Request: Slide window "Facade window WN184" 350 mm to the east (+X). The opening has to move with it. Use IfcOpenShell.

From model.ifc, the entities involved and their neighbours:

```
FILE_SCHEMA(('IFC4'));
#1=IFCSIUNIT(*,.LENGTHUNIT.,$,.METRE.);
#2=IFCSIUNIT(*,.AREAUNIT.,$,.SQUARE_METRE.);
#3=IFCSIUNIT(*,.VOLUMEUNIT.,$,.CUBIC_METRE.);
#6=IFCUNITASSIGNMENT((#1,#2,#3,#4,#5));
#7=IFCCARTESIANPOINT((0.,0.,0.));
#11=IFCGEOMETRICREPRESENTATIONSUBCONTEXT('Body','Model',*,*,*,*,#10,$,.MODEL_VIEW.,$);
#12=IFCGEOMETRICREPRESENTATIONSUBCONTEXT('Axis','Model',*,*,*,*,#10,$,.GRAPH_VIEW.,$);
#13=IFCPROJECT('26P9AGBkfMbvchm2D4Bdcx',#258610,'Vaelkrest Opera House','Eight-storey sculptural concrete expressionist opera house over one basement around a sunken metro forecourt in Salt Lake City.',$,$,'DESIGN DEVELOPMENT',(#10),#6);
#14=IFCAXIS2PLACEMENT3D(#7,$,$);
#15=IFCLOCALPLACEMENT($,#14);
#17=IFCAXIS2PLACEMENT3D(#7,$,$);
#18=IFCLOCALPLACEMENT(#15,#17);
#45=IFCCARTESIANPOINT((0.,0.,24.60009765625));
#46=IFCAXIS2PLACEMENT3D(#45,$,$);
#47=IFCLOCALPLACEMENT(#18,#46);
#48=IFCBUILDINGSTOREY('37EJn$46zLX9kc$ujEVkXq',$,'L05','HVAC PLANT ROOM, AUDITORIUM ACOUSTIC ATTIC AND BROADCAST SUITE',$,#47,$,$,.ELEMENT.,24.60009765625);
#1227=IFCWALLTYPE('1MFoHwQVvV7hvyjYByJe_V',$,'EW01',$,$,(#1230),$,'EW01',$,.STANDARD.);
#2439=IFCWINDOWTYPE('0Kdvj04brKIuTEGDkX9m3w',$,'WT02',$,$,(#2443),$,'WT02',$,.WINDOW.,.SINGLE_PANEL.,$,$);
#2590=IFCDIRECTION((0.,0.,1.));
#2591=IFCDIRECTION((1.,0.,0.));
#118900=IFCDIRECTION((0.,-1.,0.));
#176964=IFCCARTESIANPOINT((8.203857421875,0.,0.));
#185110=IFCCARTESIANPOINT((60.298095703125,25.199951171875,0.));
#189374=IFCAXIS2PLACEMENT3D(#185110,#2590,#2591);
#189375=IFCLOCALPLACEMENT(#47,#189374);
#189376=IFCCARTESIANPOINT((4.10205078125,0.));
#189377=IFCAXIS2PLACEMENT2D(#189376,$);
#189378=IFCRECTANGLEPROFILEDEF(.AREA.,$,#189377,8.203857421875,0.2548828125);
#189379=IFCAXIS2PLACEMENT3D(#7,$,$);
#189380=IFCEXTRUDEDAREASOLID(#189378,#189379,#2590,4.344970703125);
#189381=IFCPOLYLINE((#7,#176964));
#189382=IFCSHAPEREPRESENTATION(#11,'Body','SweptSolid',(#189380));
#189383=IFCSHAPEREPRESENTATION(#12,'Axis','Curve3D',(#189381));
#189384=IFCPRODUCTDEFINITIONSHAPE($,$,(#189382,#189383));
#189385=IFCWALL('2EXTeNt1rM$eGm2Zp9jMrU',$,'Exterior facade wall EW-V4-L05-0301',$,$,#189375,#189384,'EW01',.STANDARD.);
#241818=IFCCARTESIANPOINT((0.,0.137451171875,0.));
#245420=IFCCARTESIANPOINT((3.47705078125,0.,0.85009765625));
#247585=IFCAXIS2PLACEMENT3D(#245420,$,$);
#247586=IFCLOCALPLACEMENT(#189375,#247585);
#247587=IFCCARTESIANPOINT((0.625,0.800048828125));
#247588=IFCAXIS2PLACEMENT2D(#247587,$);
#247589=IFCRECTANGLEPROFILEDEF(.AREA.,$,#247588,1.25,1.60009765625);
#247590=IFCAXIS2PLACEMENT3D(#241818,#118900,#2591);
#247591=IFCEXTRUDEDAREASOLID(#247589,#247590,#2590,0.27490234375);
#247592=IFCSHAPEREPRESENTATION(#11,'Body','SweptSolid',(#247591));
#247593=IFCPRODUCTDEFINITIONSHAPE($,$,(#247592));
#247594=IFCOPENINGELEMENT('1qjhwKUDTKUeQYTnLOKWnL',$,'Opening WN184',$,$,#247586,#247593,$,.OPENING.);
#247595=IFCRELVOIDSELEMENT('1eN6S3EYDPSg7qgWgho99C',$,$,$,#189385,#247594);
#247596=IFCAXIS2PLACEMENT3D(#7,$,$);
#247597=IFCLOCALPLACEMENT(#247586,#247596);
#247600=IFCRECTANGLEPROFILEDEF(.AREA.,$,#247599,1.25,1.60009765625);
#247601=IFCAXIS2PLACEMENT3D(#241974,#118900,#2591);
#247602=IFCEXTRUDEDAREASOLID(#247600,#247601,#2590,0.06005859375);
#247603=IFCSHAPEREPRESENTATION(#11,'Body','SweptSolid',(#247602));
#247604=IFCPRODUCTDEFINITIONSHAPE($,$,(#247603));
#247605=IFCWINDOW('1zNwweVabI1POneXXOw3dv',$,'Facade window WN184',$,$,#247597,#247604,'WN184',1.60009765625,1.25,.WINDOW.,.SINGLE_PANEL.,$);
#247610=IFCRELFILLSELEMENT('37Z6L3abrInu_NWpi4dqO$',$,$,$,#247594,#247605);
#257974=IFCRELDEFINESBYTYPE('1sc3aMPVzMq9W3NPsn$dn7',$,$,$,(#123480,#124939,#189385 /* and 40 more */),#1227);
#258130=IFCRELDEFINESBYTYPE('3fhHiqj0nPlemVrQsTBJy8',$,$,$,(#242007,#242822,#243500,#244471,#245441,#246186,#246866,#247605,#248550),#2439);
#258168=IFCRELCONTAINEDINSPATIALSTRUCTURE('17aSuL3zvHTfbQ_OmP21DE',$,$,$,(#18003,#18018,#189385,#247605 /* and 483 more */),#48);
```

```python
import ifcopenshell
import ifcopenshell.api.geometry
import ifcopenshell.util.placement

model = ifcopenshell.open("model.ifc")

window = model.by_guid("1zNwweVabI1POneXXOw3dv")
opening = window.FillsVoids[0].RelatingOpeningElement
wall = opening.VoidsElements[0].RelatingBuildingElement

wall_matrix = ifcopenshell.util.placement.get_local_placement(wall.ObjectPlacement)
shift = wall_matrix[:3, 0] * 0.35
before = ifcopenshell.util.placement.get_local_placement(window.ObjectPlacement)[:3, 3].copy()

# The window is placed relative to its opening, so it follows when the opening moves.
matrix = ifcopenshell.util.placement.get_local_placement(opening.ObjectPlacement)
matrix[:3, 3] += shift
ifcopenshell.api.geometry.edit_object_placement(
    model, product=opening, matrix=matrix, is_si=False, should_transform_children=True
)

after = ifcopenshell.util.placement.get_local_placement(window.ObjectPlacement)[:3, 3]
print("window moved by", (after - before).round(3) + 0.0)

model.write("model_edited.ifc")
```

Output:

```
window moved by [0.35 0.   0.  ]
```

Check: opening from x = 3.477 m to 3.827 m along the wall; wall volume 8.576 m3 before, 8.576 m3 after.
